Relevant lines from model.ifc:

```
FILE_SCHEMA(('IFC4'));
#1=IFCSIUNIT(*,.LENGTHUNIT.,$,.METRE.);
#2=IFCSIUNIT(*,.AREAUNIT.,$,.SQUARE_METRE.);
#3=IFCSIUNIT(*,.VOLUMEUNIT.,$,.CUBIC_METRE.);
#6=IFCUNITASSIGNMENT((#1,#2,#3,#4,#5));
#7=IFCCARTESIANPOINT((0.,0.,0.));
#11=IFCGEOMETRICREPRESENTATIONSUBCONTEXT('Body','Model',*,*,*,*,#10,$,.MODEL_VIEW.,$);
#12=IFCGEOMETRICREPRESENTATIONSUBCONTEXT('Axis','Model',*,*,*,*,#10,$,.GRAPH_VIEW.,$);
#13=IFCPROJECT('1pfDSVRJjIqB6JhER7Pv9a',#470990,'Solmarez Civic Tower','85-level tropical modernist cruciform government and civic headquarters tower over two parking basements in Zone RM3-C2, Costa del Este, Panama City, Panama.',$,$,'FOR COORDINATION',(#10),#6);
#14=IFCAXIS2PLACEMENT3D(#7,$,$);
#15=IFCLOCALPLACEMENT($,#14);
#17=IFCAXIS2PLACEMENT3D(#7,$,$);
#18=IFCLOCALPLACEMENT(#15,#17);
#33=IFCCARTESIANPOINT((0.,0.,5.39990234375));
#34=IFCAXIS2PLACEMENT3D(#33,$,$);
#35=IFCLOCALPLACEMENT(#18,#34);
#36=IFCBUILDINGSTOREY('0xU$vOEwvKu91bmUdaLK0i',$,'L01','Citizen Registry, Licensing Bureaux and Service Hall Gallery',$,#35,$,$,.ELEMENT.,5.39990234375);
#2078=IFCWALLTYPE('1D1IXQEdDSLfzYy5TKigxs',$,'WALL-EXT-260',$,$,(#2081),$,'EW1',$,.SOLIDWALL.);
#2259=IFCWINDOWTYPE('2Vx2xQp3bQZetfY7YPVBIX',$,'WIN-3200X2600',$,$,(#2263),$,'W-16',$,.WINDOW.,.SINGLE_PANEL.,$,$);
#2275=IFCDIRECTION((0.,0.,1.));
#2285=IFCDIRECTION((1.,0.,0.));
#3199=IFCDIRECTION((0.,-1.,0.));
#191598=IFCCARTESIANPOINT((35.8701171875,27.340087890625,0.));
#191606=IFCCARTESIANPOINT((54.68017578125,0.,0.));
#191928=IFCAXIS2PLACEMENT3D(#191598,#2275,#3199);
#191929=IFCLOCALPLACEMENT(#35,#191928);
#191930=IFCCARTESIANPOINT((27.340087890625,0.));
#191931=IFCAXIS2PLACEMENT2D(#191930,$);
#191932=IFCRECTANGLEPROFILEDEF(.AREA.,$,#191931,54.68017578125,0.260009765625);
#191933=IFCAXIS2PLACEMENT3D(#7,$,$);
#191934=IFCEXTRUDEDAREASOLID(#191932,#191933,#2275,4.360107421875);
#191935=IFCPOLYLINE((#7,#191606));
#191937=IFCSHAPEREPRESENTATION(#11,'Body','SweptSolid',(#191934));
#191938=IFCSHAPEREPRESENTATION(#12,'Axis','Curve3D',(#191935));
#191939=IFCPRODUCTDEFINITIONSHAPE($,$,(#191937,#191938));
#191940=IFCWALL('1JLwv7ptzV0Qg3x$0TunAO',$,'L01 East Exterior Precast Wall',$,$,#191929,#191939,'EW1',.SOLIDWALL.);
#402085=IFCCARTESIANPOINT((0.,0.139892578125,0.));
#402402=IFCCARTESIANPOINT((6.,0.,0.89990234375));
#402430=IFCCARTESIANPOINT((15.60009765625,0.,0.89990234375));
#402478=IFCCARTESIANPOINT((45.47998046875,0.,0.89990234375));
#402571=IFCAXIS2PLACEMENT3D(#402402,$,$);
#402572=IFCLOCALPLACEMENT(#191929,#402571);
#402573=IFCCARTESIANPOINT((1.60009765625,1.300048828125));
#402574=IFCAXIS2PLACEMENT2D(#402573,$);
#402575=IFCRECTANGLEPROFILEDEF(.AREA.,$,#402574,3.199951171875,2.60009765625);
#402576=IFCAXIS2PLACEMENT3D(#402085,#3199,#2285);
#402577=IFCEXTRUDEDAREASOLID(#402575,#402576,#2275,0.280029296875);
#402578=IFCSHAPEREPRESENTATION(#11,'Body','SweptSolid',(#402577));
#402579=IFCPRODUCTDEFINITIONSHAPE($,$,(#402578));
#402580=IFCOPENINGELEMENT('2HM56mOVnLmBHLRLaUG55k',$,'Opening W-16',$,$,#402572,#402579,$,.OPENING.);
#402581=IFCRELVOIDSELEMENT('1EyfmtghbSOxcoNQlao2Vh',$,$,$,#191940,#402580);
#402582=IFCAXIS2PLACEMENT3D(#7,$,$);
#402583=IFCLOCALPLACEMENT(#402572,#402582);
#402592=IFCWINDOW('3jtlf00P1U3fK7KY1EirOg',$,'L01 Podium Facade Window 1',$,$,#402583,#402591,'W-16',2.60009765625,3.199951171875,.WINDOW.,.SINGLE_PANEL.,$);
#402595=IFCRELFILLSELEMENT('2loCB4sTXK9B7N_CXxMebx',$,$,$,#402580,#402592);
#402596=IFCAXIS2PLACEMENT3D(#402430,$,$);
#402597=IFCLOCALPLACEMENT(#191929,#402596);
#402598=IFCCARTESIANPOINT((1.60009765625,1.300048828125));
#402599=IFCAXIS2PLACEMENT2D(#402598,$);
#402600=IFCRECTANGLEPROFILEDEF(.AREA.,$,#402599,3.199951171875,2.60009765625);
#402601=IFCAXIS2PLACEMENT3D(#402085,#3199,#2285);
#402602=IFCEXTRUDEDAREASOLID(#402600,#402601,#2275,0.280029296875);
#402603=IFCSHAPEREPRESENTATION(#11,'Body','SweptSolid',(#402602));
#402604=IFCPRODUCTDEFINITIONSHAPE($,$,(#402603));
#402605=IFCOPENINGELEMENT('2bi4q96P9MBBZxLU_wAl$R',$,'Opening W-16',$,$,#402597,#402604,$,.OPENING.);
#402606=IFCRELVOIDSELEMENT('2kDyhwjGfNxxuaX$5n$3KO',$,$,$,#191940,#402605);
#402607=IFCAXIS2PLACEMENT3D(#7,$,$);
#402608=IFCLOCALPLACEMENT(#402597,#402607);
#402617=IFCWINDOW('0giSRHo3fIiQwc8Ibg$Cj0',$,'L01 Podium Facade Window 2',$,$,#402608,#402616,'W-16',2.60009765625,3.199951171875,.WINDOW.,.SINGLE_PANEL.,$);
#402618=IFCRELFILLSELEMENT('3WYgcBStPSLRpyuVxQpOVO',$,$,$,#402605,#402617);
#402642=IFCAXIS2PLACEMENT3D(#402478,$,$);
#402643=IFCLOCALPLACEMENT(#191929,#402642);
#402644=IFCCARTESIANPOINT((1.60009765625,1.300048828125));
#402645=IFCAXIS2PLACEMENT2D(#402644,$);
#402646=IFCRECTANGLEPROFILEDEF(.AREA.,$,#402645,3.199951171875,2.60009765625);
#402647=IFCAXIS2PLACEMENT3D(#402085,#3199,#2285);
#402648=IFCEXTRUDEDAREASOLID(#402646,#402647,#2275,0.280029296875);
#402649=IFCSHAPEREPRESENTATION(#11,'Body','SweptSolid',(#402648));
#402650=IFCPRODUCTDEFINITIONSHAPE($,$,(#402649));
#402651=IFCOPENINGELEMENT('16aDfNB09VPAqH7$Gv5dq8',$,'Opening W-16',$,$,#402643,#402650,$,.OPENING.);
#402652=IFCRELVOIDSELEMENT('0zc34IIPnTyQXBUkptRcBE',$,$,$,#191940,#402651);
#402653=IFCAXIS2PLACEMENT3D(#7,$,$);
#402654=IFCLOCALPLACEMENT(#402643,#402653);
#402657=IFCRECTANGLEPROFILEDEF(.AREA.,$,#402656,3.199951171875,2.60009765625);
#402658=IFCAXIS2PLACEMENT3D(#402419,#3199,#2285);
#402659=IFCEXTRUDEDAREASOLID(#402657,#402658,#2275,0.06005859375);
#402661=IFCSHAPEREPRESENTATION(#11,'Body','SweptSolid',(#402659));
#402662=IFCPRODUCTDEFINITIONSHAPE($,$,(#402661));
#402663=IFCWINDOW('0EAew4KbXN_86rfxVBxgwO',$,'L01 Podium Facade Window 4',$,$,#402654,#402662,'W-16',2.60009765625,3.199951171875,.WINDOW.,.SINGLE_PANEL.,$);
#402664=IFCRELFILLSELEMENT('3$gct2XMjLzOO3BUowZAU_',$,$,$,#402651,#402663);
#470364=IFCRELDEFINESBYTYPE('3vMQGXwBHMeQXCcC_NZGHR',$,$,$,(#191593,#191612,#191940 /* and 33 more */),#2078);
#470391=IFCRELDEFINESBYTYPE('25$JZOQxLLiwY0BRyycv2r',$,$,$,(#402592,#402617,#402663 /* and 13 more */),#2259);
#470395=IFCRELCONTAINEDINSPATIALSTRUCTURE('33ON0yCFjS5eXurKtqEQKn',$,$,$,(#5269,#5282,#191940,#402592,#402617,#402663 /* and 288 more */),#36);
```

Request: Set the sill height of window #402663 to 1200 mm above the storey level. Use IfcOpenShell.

```python
import numpy as np
import ifcopenshell
import ifcopenshell.api.geometry
import ifcopenshell.geom
import ifcopenshell.util.element
import ifcopenshell.util.placement
import ifcopenshell.util.shape
import ifcopenshell.util.unit

model = ifcopenshell.open("model.ifc")
unit_scale = ifcopenshell.util.unit.calculate_unit_scale(model)

window = model.by_id(402663)
opening = window.FillsVoids[0].RelatingOpeningElement
storey = ifcopenshell.util.element.get_container(window, ifc_class="IfcBuildingStorey")
level = ifcopenshell.util.placement.get_local_placement(storey.ObjectPlacement)[2, 3]

# The opening's origin need not be at the sill, so measure its lowest point.
shape = ifcopenshell.geom.create_shape(ifcopenshell.geom.settings(), opening)
bottom = ifcopenshell.util.shape.get_shape_bottom_elevation(shape, shape.geometry) / unit_scale
dz = level + 1.2 / unit_scale - bottom

shift = np.array([0.0, 0.0, dz])
# The window is placed relative to its opening, so it follows when the opening moves.
matrix = ifcopenshell.util.placement.get_local_placement(opening.ObjectPlacement)
matrix[:3, 3] += shift
ifcopenshell.api.geometry.edit_object_placement(
    model, product=opening, matrix=matrix, is_si=False, should_transform_children=True
)

print(f"moved by {dz * unit_scale:+.3f} m")

model.write("model-out.ifc")
```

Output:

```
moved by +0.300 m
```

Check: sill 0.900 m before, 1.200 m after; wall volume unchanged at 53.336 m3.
